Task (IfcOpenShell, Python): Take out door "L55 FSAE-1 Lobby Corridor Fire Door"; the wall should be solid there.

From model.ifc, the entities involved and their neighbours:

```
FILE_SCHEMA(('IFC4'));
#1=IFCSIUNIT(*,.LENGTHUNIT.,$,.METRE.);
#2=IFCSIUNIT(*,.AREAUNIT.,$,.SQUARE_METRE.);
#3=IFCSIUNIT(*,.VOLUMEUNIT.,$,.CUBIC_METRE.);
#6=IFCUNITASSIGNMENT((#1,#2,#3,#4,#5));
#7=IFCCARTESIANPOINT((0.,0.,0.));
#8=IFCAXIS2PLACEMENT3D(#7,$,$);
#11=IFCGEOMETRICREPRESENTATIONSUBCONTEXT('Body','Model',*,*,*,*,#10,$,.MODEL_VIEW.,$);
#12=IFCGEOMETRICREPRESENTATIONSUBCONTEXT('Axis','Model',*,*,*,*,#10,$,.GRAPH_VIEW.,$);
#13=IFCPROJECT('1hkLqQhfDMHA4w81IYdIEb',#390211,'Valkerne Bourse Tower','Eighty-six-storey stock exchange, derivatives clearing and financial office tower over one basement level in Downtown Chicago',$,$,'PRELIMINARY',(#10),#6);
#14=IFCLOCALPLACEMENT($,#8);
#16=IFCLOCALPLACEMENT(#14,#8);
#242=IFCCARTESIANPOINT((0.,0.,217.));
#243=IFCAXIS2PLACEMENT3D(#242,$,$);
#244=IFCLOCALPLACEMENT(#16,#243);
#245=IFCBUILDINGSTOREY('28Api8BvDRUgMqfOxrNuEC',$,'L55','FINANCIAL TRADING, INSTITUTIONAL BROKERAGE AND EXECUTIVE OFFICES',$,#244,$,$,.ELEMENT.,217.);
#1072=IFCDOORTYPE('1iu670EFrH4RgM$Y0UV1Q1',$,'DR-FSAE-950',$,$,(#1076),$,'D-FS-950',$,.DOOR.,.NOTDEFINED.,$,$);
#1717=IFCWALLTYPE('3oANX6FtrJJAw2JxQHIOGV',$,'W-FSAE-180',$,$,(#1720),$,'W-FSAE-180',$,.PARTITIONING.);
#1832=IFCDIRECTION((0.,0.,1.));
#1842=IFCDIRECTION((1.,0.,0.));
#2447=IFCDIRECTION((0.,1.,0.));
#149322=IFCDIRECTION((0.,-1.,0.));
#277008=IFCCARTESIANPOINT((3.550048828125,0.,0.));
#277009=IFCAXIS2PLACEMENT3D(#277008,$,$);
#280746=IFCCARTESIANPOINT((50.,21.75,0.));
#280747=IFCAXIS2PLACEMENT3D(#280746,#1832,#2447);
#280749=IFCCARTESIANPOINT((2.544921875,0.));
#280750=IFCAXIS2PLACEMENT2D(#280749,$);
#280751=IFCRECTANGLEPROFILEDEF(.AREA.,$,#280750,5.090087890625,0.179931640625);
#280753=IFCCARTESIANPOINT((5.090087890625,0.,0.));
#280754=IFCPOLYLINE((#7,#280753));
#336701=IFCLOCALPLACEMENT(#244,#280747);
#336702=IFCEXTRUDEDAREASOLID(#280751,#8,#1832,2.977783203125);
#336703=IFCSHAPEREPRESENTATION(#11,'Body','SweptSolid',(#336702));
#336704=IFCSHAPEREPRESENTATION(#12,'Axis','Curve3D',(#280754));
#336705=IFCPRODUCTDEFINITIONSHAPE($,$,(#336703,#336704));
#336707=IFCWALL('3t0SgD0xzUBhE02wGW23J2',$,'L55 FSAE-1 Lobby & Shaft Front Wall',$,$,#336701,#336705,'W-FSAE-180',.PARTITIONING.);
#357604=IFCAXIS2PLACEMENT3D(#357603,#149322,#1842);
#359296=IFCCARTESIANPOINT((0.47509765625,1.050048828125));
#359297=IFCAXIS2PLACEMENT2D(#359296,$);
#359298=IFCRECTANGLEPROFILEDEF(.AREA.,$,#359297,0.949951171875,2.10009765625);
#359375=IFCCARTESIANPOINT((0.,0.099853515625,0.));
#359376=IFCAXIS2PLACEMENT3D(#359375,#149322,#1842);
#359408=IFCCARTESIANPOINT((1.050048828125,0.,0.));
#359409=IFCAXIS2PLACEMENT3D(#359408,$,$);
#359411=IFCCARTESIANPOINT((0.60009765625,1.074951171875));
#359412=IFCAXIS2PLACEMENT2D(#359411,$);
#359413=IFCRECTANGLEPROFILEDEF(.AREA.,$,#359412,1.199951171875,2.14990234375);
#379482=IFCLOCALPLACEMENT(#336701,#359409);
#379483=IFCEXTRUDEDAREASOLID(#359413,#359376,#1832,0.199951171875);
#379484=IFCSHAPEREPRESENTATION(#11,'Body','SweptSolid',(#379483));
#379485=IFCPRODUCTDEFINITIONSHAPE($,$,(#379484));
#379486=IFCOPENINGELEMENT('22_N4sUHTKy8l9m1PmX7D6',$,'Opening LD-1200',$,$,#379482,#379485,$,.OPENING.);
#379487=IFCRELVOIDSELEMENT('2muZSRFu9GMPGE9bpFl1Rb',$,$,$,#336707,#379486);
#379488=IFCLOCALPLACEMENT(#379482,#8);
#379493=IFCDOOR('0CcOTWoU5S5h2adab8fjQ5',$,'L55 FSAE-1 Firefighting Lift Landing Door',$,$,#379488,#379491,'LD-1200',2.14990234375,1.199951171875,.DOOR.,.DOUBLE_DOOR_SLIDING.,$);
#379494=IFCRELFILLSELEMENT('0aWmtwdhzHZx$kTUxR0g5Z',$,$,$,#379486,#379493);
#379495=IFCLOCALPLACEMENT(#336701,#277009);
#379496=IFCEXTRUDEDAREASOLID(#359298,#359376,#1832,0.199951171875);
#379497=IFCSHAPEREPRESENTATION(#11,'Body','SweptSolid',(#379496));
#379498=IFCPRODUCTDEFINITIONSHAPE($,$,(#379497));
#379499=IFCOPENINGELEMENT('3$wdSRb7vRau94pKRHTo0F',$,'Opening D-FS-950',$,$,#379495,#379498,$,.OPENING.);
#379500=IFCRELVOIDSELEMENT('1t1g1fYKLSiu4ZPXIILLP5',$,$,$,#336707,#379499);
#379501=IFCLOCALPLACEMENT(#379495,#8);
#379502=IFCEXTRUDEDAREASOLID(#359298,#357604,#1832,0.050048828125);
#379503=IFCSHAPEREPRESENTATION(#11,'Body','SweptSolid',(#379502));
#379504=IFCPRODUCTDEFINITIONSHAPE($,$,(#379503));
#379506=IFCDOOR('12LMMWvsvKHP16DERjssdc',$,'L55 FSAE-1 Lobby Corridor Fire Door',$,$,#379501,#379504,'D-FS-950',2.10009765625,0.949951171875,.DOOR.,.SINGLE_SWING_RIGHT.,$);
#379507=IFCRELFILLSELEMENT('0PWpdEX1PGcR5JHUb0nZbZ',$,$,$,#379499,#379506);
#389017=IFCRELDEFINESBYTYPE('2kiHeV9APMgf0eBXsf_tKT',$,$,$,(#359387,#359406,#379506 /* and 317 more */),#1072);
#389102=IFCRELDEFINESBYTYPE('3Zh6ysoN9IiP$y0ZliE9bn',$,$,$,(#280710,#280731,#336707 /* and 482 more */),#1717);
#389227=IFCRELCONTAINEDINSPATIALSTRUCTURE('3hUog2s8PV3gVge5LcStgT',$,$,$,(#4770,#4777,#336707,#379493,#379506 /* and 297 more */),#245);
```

```python
import ifcopenshell
import ifcopenshell.api.feature
import ifcopenshell.api.root
import ifcopenshell.geom
import ifcopenshell.util.shape

model = ifcopenshell.open("model.ifc")
settings = ifcopenshell.geom.settings()


def volume(element):
    """Net volume in cubic metres, openings subtracted."""
    shape = ifcopenshell.geom.create_shape(settings, element)
    return ifcopenshell.util.shape.get_volume(shape.geometry)


door = model.by_guid("12LMMWvsvKHP16DERjssdc")
opening = door.FillsVoids[0].RelatingOpeningElement
wall = opening.VoidsElements[0].RelatingBuildingElement
before = volume(wall)

ifcopenshell.api.root.remove_product(model, product=door)
ifcopenshell.api.feature.remove_feature(model, feature=opening)

after = volume(wall)

print(f"wall volume {before:.3f} -> {after:.3f} m3")

model.write("model_edited.ifc")
```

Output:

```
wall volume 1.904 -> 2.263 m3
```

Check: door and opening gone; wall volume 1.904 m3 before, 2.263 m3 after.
